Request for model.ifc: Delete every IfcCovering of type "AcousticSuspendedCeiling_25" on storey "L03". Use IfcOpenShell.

First a look at what the model holds.

```python
import ifcopenshell
import ifcopenshell.util.element

model = ifcopenshell.open("model.ifc")
print(model.schema)
storey = next(s for s in model.by_type("IfcBuildingStorey") if s.Name == "L03")
coverings = [e for e in ifcopenshell.util.element.get_decomposition(storey) if e.is_a("IfcCovering")]
seen = {}
for e in coverings:
    element_type = ifcopenshell.util.element.get_type(e)
    name = element_type.Name if element_type not in (None, e) else None
    seen[name] = seen.get(name, 0) + 1
for name, count in sorted(seen.items(), key=str):
    print(count, "x", name)
```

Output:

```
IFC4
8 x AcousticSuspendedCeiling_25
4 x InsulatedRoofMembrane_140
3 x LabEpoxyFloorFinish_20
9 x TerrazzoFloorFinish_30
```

```python
import ifcopenshell
import ifcopenshell.api.root
import ifcopenshell.util.element

model = ifcopenshell.open("model.ifc")

storey = next(s for s in model.by_type("IfcBuildingStorey") if s.Name == "L03")
coverings = [e for e in ifcopenshell.util.element.get_decomposition(storey) if e.is_a("IfcCovering")]
targets = [e for e in coverings if (t := ifcopenshell.util.element.get_type(e)) not in (None, e) and t.Name == "AcousticSuspendedCeiling_25"]

for e in targets:
    ifcopenshell.api.root.remove_product(model, product=e)
print(len(targets), "removed")

model.write("model_v2.ifc")
```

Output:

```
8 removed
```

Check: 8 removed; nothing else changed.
